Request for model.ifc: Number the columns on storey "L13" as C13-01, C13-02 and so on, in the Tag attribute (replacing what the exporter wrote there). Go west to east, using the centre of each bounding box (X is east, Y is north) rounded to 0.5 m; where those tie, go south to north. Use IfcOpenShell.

First a look at what the model holds.

```python
import ifcopenshell
import ifcopenshell.util.element
import ifcopenshell.util.placement

model = ifcopenshell.open("model.ifc")
print(model.schema)
storey = next(s for s in model.by_type("IfcBuildingStorey") if s.Name == "L13")
columns = [e for e in ifcopenshell.util.element.get_decomposition(storey) if e.is_a("IfcColumn")]
for e in sorted(columns, key=lambda e: e.id()):
    origin = ifcopenshell.util.placement.get_local_placement(e.ObjectPlacement)[:3, 3]
    print(e.id(), e.Tag, e.Name, origin.round(2) + 0.0, sep=" | ")
```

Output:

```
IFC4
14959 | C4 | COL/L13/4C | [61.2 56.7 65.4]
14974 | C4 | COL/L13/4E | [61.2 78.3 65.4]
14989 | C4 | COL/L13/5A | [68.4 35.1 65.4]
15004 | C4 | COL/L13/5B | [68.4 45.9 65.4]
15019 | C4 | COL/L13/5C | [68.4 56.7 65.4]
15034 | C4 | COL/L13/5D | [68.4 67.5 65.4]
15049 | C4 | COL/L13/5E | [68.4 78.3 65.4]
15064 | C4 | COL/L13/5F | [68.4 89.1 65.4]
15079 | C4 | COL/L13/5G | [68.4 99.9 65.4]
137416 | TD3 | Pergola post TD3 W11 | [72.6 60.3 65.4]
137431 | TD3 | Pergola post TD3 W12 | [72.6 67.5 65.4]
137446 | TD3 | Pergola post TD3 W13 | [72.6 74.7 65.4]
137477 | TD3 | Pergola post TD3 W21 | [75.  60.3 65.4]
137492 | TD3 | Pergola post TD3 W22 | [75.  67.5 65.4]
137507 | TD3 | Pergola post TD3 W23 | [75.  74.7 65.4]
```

```python
import ifcopenshell
import ifcopenshell.geom
import ifcopenshell.util.element
import ifcopenshell.util.shape

model = ifcopenshell.open("model.ifc")
settings = ifcopenshell.geom.settings()
settings.set("use-world-coords", True)


def centre(element):
    shape = ifcopenshell.geom.create_shape(settings, element)
    return ifcopenshell.util.shape.get_bbox_centroid(shape.geometry)


storey = next(s for s in model.by_type("IfcBuildingStorey") if s.Name == "L13")
columns = [e for e in ifcopenshell.util.element.get_decomposition(storey) if e.is_a("IfcColumn")]

# Insertion points can sit at a corner or the storey origin, so sort by the geometry (in metres).
centres = {e: centre(e) for e in columns}
columns.sort(key=lambda e: (round(centres[e][0] / 0.5), centres[e][1]))

for i, e in enumerate(columns, start=1):
    number = f"C13-{i:02d}"
    e.Tag = number
    print(e.id(), number)

model.write("model_rev.ifc")
```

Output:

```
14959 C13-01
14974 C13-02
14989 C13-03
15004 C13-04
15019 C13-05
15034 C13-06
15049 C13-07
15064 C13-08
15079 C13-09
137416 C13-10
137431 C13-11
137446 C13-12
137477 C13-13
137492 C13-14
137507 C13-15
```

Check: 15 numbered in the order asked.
